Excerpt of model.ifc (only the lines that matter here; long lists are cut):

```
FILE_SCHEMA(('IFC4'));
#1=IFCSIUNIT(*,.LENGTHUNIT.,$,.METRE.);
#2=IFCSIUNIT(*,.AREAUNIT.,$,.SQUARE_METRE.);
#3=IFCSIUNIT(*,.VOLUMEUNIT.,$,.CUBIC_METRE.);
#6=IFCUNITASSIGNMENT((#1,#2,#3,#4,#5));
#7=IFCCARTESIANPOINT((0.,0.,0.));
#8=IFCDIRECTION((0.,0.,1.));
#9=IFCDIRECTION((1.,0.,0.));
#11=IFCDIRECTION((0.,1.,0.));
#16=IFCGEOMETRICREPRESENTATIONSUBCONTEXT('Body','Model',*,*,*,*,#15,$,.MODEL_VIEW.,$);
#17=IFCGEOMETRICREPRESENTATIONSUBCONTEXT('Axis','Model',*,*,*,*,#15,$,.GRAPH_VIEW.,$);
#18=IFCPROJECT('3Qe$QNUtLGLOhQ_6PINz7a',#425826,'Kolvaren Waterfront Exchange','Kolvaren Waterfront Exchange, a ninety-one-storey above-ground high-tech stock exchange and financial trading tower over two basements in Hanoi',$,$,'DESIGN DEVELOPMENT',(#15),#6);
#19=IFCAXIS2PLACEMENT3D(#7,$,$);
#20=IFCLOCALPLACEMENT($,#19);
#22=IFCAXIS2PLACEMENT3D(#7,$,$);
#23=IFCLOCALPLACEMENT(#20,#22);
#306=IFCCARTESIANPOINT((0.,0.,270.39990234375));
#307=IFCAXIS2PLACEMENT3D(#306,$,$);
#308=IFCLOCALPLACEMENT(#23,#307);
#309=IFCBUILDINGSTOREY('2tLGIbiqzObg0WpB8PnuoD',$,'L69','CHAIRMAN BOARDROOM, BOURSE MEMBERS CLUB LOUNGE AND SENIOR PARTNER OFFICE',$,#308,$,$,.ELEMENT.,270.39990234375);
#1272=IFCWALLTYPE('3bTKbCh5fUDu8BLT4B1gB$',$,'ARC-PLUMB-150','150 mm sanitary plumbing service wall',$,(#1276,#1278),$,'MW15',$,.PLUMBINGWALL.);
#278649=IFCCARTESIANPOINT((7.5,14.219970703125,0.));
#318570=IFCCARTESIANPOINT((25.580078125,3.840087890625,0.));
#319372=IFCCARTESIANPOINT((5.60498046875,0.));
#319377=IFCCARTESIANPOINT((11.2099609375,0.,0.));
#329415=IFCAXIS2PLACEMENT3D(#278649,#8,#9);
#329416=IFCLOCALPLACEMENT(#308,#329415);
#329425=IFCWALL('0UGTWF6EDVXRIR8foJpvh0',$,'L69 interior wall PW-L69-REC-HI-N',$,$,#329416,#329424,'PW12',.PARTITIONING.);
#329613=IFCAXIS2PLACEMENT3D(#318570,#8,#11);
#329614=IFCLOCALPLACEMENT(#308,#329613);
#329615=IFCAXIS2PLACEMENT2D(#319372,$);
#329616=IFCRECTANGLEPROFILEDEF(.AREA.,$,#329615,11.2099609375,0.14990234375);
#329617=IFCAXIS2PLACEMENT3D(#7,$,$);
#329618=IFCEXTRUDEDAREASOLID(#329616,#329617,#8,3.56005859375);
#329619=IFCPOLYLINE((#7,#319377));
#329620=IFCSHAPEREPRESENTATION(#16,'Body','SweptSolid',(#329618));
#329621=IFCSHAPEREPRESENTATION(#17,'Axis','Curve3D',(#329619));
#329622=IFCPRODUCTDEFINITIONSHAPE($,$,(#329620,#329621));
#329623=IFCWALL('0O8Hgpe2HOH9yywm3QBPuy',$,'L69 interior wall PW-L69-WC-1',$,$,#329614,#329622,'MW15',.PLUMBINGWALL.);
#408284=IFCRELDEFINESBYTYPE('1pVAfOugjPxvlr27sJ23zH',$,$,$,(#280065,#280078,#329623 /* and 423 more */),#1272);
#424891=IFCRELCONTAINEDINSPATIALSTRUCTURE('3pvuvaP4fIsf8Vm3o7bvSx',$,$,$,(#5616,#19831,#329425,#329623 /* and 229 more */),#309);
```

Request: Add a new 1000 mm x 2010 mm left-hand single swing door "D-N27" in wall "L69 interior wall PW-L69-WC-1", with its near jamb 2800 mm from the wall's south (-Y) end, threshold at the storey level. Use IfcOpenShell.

```python
import numpy as np
import ifcopenshell
import ifcopenshell.api.feature
import ifcopenshell.api.geometry
import ifcopenshell.api.root
import ifcopenshell.api.spatial
import ifcopenshell.geom
import ifcopenshell.util.element
import ifcopenshell.util.placement
import ifcopenshell.util.representation
import ifcopenshell.util.shape
import ifcopenshell.util.unit

model = ifcopenshell.open("model.ifc")
unit_scale = ifcopenshell.util.unit.calculate_unit_scale(model)
settings = ifcopenshell.geom.settings()


def volume(element):
    """Net volume in cubic metres, openings subtracted."""
    shape = ifcopenshell.geom.create_shape(settings, element)
    return ifcopenshell.util.shape.get_volume(shape.geometry)


wall = model.by_id(329623)
storey = ifcopenshell.util.element.get_container(wall, ifc_class="IfcBuildingStorey")
context = ifcopenshell.util.representation.get_context(model, "Model", "Body", "MODEL_VIEW")
before = volume(wall)

width, height, from_end, sill = 1, 2.01, 2.8, 0.0  # metres

# The wall runs along its own X axis, and the end named is its -X end.
wall_shape = ifcopenshell.geom.create_shape(settings, wall)
x, y, z = ifcopenshell.util.shape.get_vertices(wall_shape.geometry).T
start = x.min() + from_end
face, thickness = float(y.min()), float(y.max() - y.min())
wall_matrix = ifcopenshell.util.placement.get_local_placement(wall.ObjectPlacement)
level = ifcopenshell.util.placement.get_local_placement(storey.ObjectPlacement)[2, 3]


def in_wall(x, y):
    """Placement at x, y metres in the wall's axes, at sill height."""
    matrix = wall_matrix.copy()
    matrix[:, 3] = wall_matrix @ np.array([x / unit_scale, y / unit_scale, 0.0, 1.0])
    matrix[2, 3] = level + sill / unit_scale
    return matrix


# Opening: a box that overshoots both wall faces by 50 mm.
opening = ifcopenshell.api.root.create_entity(model, ifc_class="IfcOpeningElement", predefined_type="OPENING")
box = ifcopenshell.api.geometry.add_wall_representation(
    model, context=context, length=width, height=height, thickness=thickness + 0.1
)
ifcopenshell.api.geometry.assign_representation(model, product=opening, representation=box)
ifcopenshell.api.geometry.edit_object_placement(model, product=opening, matrix=in_wall(start, face - 0.05), is_si=False)
ifcopenshell.api.feature.add_feature(model, feature=opening, element=wall)

door = ifcopenshell.api.root.create_entity(model, ifc_class="IfcDoor", name="D-N27", predefined_type="DOOR")
door.OverallWidth, door.OverallHeight = width / unit_scale, height / unit_scale
door.OperationType = "SINGLE_SWING_LEFT"
body = ifcopenshell.api.geometry.add_door_representation(
    model,
    context=context,
    overall_width=door.OverallWidth,
    overall_height=door.OverallHeight,
    operation_type="SINGLE_SWING_LEFT",
    lining_properties={"LiningDepth": thickness / unit_scale, "ThresholdDepth": thickness / unit_scale},
)
ifcopenshell.api.geometry.assign_representation(model, product=door, representation=body)
ifcopenshell.api.spatial.assign_container(model, products=[door], relating_structure=storey)
ifcopenshell.api.feature.add_filling(model, opening=opening, element=door)

# The lining spans the wall, so the door starts at the wall face.
ifcopenshell.api.geometry.edit_object_placement(model, product=door, matrix=in_wall(start, face), is_si=False)

after = volume(wall)

print(f"wall volume {before:.3f} -> {after:.3f} m3")

model.write("model-out.ifc")
```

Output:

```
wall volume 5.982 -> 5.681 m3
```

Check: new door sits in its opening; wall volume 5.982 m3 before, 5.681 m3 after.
